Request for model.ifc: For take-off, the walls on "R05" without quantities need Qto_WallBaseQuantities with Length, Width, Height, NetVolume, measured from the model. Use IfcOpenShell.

First a look at what the model holds.

```python
import ifcopenshell
import ifcopenshell.util.element
import ifcopenshell.util.unit

model = ifcopenshell.open("model.ifc")
print(model.schema)
for unit_type in ("LENGTHUNIT", "AREAUNIT", "VOLUMEUNIT"):
    print(unit_type, ifcopenshell.util.unit.calculate_unit_scale(model, unit_type))
storey = next(s for s in model.by_type("IfcBuildingStorey") if s.Name == "R05")
walls = [e for e in ifcopenshell.util.element.get_decomposition(storey) if e.is_a("IfcWall")]
for e in sorted(walls, key=lambda e: e.id()):
    print(e.id(), e.is_a(), e.Name, list(ifcopenshell.util.element.get_psets(e, qtos_only=True)), sep=" | ")
```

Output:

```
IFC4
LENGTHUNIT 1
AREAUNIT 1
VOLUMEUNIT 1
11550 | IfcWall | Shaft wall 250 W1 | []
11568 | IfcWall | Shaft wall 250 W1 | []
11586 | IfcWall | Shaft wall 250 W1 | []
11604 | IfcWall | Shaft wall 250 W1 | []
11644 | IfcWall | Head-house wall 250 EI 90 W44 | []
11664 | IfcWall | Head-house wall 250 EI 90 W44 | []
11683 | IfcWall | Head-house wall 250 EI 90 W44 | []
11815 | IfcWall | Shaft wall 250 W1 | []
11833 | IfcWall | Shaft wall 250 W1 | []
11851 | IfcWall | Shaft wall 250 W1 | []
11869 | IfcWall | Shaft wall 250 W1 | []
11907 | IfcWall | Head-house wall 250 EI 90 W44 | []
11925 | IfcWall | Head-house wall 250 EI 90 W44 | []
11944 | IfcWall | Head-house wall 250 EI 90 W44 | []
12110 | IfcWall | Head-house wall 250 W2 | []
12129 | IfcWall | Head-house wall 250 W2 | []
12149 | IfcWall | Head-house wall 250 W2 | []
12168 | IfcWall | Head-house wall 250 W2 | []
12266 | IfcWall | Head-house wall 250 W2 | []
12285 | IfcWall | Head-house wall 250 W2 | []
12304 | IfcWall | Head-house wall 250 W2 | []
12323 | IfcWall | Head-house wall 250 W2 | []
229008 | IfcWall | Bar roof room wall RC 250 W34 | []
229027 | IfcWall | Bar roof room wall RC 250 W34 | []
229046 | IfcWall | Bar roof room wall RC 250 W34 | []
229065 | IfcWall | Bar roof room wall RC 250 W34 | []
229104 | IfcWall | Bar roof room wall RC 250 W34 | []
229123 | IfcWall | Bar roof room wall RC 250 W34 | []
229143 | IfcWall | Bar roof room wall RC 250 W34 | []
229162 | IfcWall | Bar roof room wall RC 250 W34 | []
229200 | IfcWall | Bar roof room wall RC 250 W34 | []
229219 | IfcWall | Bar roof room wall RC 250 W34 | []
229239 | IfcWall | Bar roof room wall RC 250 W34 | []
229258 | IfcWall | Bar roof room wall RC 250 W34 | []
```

```python
import ifcopenshell
import ifcopenshell.api.pset
import ifcopenshell.geom
import ifcopenshell.util.element
import ifcopenshell.util.shape
import ifcopenshell.util.unit

model = ifcopenshell.open("model.ifc")
unit_scale = ifcopenshell.util.unit.calculate_unit_scale(model)
volume_scale = ifcopenshell.util.unit.calculate_unit_scale(model, "VOLUMEUNIT")
settings = ifcopenshell.geom.settings()

storey = next(s for s in model.by_type("IfcBuildingStorey") if s.Name == "R05")
walls = [e for e in ifcopenshell.util.element.get_decomposition(storey) if e.is_a("IfcWall")]

for e in sorted(walls, key=lambda e: e.id()):
    if ifcopenshell.util.element.get_psets(e, qtos_only=True, should_inherit=False):
        continue
    # Geometry comes back in metres, in the element's own axes.
    shape = ifcopenshell.geom.create_shape(settings, e)
    values = {
        "Length": ifcopenshell.util.shape.get_x(shape.geometry) / unit_scale,
        "Width": ifcopenshell.util.shape.get_y(shape.geometry) / unit_scale,
        "Height": ifcopenshell.util.shape.get_z(shape.geometry) / unit_scale,
        "NetVolume": ifcopenshell.util.shape.get_volume(shape.geometry) / volume_scale,
    }
    qto = ifcopenshell.api.pset.add_qto(model, product=e, name="Qto_WallBaseQuantities")
    ifcopenshell.api.pset.edit_qto(model, qto=qto, properties=values)
    print(e.id(), {k: round(v, 3) for k, v in values.items()})

model.write("model_updated.ifc")
```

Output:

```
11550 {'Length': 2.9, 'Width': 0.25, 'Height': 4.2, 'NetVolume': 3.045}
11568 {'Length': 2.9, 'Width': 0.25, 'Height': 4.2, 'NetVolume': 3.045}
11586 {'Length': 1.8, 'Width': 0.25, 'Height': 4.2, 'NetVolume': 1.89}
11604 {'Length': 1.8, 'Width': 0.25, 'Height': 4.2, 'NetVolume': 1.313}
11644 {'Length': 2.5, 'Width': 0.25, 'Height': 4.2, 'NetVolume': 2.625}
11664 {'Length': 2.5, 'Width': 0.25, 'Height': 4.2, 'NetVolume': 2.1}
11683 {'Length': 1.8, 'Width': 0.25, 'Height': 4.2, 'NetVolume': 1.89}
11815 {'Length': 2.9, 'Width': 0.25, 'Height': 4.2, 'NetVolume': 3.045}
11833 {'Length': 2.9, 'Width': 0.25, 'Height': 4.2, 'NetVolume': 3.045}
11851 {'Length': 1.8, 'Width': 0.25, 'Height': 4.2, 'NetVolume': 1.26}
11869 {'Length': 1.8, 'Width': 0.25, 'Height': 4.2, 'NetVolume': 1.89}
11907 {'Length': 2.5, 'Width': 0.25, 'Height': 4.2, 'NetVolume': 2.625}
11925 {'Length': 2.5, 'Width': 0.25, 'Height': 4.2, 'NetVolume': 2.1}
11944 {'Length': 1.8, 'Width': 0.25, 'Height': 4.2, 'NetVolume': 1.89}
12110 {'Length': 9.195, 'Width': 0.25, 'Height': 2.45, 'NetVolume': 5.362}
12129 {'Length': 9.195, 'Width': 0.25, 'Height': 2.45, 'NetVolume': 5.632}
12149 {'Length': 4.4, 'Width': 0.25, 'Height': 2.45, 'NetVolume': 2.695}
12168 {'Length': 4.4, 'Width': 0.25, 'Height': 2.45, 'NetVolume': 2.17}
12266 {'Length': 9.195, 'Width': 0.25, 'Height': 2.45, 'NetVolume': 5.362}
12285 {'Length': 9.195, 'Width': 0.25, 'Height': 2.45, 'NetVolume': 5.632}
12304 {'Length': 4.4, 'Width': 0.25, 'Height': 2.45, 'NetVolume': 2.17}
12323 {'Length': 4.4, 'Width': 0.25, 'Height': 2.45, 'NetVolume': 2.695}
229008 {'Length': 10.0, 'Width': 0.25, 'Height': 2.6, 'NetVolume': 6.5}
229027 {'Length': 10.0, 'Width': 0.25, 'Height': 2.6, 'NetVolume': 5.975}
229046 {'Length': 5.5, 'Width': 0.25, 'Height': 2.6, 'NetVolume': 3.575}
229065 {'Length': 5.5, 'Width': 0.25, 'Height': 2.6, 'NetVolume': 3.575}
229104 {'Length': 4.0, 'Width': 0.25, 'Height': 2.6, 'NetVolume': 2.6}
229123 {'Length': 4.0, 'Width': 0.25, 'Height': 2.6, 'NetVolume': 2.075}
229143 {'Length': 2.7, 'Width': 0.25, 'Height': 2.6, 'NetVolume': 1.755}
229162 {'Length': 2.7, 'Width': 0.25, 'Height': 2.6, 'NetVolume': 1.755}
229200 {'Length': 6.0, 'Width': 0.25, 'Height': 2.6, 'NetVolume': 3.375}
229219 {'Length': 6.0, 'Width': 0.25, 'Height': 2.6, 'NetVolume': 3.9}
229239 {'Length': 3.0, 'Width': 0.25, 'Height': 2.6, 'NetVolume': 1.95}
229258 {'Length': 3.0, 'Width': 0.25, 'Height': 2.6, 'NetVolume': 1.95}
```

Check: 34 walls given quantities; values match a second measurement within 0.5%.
